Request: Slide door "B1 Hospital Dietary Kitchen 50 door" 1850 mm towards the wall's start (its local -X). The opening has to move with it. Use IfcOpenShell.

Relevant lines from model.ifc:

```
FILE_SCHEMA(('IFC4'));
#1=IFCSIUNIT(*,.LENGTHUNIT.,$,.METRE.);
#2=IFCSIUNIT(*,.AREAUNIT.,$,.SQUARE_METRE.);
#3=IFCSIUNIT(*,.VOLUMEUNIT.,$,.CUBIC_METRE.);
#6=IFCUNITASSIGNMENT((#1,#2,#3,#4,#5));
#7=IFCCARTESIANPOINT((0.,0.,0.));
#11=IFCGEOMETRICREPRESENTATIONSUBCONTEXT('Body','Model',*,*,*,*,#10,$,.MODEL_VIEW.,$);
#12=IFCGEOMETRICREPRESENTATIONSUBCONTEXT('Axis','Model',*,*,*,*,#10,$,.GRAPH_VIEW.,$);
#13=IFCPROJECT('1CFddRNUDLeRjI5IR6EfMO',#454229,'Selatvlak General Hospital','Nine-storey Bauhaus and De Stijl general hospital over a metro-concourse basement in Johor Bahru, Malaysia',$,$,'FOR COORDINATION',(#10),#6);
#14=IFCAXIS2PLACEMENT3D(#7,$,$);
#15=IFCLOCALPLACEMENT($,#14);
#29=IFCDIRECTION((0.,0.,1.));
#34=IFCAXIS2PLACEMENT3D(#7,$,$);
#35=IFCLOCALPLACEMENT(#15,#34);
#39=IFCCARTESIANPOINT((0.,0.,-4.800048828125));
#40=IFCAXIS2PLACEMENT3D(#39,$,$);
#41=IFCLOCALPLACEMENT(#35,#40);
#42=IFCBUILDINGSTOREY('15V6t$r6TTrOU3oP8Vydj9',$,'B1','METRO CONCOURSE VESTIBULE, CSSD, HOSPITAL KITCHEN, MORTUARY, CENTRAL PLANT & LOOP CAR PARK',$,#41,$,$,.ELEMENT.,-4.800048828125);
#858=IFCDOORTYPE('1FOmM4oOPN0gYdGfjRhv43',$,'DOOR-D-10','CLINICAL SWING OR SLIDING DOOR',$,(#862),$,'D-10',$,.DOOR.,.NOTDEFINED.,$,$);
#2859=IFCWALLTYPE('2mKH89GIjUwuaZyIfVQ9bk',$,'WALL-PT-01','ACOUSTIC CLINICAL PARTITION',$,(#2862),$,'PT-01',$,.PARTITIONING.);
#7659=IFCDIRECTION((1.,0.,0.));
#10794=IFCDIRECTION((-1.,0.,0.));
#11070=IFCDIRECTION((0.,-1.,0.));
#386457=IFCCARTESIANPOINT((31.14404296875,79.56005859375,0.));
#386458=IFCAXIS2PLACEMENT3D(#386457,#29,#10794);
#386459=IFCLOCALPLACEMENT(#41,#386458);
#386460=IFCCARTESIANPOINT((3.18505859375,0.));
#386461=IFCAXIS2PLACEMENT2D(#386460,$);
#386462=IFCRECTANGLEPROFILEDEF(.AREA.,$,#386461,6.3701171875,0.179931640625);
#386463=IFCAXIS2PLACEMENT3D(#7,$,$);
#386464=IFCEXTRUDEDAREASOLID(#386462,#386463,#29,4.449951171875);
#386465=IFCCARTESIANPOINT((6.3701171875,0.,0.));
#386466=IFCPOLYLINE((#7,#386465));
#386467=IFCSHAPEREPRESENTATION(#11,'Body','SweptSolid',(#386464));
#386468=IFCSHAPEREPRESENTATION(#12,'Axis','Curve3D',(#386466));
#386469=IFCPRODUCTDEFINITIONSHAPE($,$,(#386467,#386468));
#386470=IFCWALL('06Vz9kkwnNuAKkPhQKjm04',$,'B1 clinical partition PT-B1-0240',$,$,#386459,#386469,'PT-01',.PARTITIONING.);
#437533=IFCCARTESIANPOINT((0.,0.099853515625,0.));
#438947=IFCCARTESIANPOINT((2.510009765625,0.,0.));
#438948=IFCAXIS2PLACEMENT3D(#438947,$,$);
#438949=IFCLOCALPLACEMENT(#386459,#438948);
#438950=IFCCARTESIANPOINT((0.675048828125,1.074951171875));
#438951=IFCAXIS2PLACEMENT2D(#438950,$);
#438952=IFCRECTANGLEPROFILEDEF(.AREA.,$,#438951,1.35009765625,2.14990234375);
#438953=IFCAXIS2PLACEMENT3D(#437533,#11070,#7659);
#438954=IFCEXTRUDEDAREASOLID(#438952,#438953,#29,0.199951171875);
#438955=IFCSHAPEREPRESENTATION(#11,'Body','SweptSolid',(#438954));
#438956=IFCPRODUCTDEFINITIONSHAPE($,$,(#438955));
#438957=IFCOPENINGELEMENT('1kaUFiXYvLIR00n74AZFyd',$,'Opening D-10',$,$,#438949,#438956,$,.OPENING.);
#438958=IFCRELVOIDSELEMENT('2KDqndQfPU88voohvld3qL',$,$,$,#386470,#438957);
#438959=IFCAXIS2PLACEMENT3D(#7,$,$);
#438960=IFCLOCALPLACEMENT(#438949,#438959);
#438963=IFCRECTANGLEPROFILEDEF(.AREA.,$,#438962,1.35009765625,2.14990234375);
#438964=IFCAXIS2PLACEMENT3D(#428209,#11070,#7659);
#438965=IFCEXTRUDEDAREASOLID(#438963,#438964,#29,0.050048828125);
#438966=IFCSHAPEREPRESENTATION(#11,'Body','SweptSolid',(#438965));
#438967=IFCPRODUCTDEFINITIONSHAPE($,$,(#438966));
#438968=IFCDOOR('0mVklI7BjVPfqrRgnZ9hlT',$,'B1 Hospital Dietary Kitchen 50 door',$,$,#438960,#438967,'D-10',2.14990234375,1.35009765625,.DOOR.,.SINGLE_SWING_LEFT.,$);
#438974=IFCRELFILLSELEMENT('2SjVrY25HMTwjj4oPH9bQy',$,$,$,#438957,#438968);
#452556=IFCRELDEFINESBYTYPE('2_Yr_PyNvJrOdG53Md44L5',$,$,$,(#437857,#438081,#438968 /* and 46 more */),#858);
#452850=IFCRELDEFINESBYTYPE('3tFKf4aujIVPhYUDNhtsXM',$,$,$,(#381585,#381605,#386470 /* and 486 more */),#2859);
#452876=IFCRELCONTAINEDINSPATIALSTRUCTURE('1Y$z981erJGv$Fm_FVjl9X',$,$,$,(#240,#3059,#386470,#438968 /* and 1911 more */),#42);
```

```python
import ifcopenshell
import ifcopenshell.api.geometry
import ifcopenshell.util.placement
import ifcopenshell.util.unit

model = ifcopenshell.open("model.ifc")
unit_scale = ifcopenshell.util.unit.calculate_unit_scale(model)

door = model.by_guid("0mVklI7BjVPfqrRgnZ9hlT")
opening = door.FillsVoids[0].RelatingOpeningElement
wall = opening.VoidsElements[0].RelatingBuildingElement

wall_matrix = ifcopenshell.util.placement.get_local_placement(wall.ObjectPlacement)
shift = wall_matrix[:3, 0] * -1.85 / unit_scale
before = ifcopenshell.util.placement.get_local_placement(door.ObjectPlacement)[:3, 3].copy()

# The door is placed relative to its opening, so it follows when the opening moves.
matrix = ifcopenshell.util.placement.get_local_placement(opening.ObjectPlacement)
matrix[:3, 3] += shift
ifcopenshell.api.geometry.edit_object_placement(
    model, product=opening, matrix=matrix, is_si=False, should_transform_children=True
)

after = ifcopenshell.util.placement.get_local_placement(door.ObjectPlacement)[:3, 3]
print("door moved by", (after - before).round(3) + 0.0)

model.write("model_rev.ifc")
```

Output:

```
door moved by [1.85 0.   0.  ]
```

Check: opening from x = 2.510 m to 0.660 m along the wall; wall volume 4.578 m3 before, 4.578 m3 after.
